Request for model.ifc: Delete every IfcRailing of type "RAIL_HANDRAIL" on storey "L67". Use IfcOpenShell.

First a look at what the model holds.

```python
import ifcopenshell
import ifcopenshell.util.element

model = ifcopenshell.open("model.ifc")
print(model.schema)
storey = next(s for s in model.by_type("IfcBuildingStorey") if s.Name == "L67")
railings = [e for e in ifcopenshell.util.element.get_decomposition(storey) if e.is_a("IfcRailing")]
seen = {}
for e in railings:
    element_type = ifcopenshell.util.element.get_type(e)
    name = element_type.Name if element_type not in (None, e) else None
    seen[name] = seen.get(name, 0) + 1
for name, count in sorted(seen.items(), key=str):
    print(count, "x", name)
```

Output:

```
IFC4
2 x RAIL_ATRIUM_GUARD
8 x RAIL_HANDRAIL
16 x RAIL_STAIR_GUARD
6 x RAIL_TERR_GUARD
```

```python
import ifcopenshell
import ifcopenshell.api.root
import ifcopenshell.util.element

model = ifcopenshell.open("model.ifc")

storey = next(s for s in model.by_type("IfcBuildingStorey") if s.Name == "L67")
railings = [e for e in ifcopenshell.util.element.get_decomposition(storey) if e.is_a("IfcRailing")]
targets = [e for e in railings if (t := ifcopenshell.util.element.get_type(e)) not in (None, e) and t.Name == "RAIL_HANDRAIL"]

for e in targets:
    ifcopenshell.api.root.remove_product(model, product=e)
print(len(targets), "removed")

model.write("model_updated.ifc")
```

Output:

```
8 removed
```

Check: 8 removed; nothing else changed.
